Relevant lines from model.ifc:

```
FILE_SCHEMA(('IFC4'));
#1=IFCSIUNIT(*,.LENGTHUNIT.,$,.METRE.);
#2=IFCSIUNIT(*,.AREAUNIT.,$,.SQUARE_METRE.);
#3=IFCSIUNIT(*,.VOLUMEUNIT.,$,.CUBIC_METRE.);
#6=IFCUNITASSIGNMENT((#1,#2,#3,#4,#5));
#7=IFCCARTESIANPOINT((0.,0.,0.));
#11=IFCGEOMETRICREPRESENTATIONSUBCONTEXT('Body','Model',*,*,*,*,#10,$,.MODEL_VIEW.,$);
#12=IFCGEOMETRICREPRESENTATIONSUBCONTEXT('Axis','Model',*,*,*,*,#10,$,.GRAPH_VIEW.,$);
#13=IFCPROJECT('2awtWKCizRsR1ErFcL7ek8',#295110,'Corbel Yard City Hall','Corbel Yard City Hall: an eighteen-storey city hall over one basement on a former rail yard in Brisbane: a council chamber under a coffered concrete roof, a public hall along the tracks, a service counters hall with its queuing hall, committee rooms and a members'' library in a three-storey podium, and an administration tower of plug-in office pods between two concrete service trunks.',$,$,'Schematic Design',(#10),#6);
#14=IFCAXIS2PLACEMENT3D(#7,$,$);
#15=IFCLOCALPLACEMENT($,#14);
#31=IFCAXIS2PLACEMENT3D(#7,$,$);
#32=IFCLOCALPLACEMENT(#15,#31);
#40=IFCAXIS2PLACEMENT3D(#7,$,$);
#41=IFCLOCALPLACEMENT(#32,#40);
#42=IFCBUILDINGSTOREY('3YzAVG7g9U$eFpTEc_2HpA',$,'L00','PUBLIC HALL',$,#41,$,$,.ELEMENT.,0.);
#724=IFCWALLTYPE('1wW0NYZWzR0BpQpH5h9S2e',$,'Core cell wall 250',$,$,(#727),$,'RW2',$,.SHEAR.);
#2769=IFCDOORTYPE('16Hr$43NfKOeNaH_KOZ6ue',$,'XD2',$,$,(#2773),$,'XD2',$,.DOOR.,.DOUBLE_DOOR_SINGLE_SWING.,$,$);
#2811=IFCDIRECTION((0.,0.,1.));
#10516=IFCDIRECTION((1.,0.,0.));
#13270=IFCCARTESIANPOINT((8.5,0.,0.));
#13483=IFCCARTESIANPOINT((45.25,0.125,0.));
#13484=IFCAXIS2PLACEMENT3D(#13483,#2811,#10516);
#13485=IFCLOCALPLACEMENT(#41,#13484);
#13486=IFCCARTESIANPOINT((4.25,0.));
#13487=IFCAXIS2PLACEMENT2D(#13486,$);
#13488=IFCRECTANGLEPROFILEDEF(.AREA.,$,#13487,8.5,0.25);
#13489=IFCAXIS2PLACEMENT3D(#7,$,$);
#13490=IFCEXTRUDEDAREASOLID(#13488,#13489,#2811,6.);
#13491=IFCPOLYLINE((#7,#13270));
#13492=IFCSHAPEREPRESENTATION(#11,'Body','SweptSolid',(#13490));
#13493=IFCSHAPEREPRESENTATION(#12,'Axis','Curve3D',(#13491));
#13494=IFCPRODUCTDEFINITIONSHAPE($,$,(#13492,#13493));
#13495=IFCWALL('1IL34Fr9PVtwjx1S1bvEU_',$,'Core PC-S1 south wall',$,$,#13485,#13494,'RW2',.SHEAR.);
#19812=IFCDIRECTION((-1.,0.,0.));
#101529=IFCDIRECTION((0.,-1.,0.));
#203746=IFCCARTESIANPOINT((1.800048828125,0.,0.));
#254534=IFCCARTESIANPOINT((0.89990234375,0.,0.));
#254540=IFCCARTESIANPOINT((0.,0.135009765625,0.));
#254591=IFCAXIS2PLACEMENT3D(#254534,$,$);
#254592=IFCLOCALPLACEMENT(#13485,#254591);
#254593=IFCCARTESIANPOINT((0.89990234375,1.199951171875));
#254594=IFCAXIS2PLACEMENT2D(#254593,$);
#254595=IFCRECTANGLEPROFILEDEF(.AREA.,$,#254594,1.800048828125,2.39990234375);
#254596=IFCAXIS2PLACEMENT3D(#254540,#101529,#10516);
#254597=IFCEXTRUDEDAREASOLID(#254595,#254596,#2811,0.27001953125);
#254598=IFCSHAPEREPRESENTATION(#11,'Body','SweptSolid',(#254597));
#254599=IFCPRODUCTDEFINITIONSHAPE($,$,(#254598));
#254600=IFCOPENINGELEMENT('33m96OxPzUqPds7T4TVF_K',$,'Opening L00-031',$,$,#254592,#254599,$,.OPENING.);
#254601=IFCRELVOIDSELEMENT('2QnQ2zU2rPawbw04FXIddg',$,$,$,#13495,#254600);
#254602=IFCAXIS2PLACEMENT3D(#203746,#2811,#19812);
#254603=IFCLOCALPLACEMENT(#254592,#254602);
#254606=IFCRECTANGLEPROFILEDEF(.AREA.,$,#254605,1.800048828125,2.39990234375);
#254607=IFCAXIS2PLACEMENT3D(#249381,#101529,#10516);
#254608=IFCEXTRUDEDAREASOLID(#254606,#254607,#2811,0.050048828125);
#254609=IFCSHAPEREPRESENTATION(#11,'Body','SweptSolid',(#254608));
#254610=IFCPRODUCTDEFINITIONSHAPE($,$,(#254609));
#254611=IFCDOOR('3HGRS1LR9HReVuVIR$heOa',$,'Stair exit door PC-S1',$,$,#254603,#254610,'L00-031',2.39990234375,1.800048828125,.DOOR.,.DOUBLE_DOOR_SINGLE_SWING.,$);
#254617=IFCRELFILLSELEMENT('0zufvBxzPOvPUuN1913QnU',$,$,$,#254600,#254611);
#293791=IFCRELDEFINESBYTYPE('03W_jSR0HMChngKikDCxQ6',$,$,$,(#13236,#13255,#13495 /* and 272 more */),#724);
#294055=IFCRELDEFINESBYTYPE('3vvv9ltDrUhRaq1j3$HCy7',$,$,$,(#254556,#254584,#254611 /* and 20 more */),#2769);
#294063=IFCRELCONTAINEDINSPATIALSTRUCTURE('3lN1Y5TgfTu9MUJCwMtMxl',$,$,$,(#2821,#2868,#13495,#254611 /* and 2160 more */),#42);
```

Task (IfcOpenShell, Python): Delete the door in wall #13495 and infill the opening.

```python
import ifcopenshell
import ifcopenshell.api.feature
import ifcopenshell.api.root
import ifcopenshell.geom
import ifcopenshell.util.shape

model = ifcopenshell.open("model.ifc")
settings = ifcopenshell.geom.settings()


def volume(element):
    """Net volume in cubic metres, openings subtracted."""
    shape = ifcopenshell.geom.create_shape(settings, element)
    return ifcopenshell.util.shape.get_volume(shape.geometry)


door = model.by_guid("3HGRS1LR9HReVuVIR$heOa")
opening = door.FillsVoids[0].RelatingOpeningElement
wall = opening.VoidsElements[0].RelatingBuildingElement
before = volume(wall)

ifcopenshell.api.root.remove_product(model, product=door)
ifcopenshell.api.feature.remove_feature(model, feature=opening)

after = volume(wall)

print(f"wall volume {before:.3f} -> {after:.3f} m3")

model.write("model_v2.ifc")
```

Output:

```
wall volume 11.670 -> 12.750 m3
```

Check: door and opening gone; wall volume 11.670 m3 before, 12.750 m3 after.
